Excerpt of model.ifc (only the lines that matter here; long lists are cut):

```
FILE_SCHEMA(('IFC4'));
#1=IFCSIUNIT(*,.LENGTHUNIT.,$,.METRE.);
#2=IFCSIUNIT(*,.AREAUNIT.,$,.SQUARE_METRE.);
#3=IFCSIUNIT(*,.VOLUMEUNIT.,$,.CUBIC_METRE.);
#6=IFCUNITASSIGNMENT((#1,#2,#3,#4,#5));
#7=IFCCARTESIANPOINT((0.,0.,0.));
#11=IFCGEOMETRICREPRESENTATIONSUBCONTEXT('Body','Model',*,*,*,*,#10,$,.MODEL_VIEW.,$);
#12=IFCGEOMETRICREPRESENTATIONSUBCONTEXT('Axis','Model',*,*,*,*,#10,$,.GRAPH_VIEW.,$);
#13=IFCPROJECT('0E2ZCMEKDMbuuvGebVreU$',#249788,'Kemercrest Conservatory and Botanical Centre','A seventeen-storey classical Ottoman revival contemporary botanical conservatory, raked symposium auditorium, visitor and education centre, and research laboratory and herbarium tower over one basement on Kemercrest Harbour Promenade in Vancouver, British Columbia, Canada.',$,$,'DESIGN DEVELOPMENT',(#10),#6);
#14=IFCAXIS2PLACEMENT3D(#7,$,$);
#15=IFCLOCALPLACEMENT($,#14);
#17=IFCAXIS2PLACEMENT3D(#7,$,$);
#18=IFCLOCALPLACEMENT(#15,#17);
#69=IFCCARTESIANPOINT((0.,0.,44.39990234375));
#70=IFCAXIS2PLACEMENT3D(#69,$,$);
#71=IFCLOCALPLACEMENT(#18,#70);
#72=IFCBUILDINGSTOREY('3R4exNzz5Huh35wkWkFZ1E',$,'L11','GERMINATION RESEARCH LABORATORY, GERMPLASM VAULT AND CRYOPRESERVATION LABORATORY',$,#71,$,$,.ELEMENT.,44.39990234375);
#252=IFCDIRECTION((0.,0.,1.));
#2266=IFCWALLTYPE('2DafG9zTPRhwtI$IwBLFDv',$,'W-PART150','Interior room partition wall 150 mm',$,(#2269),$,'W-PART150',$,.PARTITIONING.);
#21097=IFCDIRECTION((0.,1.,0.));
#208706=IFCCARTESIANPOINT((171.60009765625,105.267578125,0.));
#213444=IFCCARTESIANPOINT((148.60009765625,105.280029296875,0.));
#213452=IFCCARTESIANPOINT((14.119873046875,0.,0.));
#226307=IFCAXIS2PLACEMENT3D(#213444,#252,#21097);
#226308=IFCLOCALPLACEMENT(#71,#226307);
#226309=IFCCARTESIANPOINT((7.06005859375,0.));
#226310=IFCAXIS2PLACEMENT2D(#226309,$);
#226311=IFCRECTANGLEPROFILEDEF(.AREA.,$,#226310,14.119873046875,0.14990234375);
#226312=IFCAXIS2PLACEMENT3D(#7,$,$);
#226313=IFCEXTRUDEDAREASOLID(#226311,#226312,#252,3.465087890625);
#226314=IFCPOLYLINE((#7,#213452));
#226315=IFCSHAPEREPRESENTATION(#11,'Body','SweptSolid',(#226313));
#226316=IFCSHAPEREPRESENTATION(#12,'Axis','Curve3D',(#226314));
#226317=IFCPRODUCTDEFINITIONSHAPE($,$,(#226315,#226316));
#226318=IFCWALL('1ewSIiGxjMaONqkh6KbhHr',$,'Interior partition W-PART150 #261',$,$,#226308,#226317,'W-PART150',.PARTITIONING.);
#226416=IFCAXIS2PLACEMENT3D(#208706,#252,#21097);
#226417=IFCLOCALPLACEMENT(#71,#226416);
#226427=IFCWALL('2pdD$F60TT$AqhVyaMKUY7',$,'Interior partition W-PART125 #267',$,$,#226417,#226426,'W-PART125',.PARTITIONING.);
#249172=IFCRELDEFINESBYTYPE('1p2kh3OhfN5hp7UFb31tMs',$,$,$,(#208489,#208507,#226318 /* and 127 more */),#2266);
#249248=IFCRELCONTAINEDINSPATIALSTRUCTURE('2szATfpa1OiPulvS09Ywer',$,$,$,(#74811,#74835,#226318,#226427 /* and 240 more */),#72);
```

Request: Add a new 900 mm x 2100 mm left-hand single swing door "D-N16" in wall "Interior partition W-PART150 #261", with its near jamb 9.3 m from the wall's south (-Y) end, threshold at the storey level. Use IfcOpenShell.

```python
import numpy as np
import ifcopenshell
import ifcopenshell.api.feature
import ifcopenshell.api.geometry
import ifcopenshell.api.root
import ifcopenshell.api.spatial
import ifcopenshell.geom
import ifcopenshell.util.element
import ifcopenshell.util.placement
import ifcopenshell.util.representation
import ifcopenshell.util.shape
import ifcopenshell.util.unit

model = ifcopenshell.open("model.ifc")
unit_scale = ifcopenshell.util.unit.calculate_unit_scale(model)
settings = ifcopenshell.geom.settings()


def volume(element):
    """Net volume in cubic metres, openings subtracted."""
    shape = ifcopenshell.geom.create_shape(settings, element)
    return ifcopenshell.util.shape.get_volume(shape.geometry)


wall = model.by_guid("1ewSIiGxjMaONqkh6KbhHr")
storey = ifcopenshell.util.element.get_container(wall, ifc_class="IfcBuildingStorey")
context = ifcopenshell.util.representation.get_context(model, "Model", "Body", "MODEL_VIEW")
before = volume(wall)

width, height, from_end, sill = 0.9, 2.1, 9.3, 0.0  # metres

# The wall runs along its own X axis, and the end named is its -X end.
wall_shape = ifcopenshell.geom.create_shape(settings, wall)
x, y, z = ifcopenshell.util.shape.get_vertices(wall_shape.geometry).T
start = x.min() + from_end
face, thickness = float(y.min()), float(y.max() - y.min())
wall_matrix = ifcopenshell.util.placement.get_local_placement(wall.ObjectPlacement)
level = ifcopenshell.util.placement.get_local_placement(storey.ObjectPlacement)[2, 3]


def in_wall(x, y):
    """Placement at x, y metres in the wall's axes, at sill height."""
    matrix = wall_matrix.copy()
    matrix[:, 3] = wall_matrix @ np.array([x / unit_scale, y / unit_scale, 0.0, 1.0])
    matrix[2, 3] = level + sill / unit_scale
    return matrix


# Opening: a box that overshoots both wall faces by 50 mm.
opening = ifcopenshell.api.root.create_entity(model, ifc_class="IfcOpeningElement", predefined_type="OPENING")
box = ifcopenshell.api.geometry.add_wall_representation(
    model, context=context, length=width, height=height, thickness=thickness + 0.1
)
ifcopenshell.api.geometry.assign_representation(model, product=opening, representation=box)
ifcopenshell.api.geometry.edit_object_placement(model, product=opening, matrix=in_wall(start, face - 0.05), is_si=False)
ifcopenshell.api.feature.add_feature(model, feature=opening, element=wall)

door = ifcopenshell.api.root.create_entity(model, ifc_class="IfcDoor", name="D-N16", predefined_type="DOOR")
door.OverallWidth, door.OverallHeight = width / unit_scale, height / unit_scale
door.OperationType = "SINGLE_SWING_LEFT"
body = ifcopenshell.api.geometry.add_door_representation(
    model,
    context=context,
    overall_width=door.OverallWidth,
    overall_height=door.OverallHeight,
    operation_type="SINGLE_SWING_LEFT",
    lining_properties={"LiningDepth": thickness / unit_scale, "ThresholdDepth": thickness / unit_scale},
)
ifcopenshell.api.geometry.assign_representation(model, product=door, representation=body)
ifcopenshell.api.spatial.assign_container(model, products=[door], relating_structure=storey)
ifcopenshell.api.feature.add_filling(model, opening=opening, element=door)

# The lining spans the wall, so the door starts at the wall face.
ifcopenshell.api.geometry.edit_object_placement(model, product=door, matrix=in_wall(start, face), is_si=False)

after = volume(wall)

print(f"wall volume {before:.3f} -> {after:.3f} m3")

model.write("model_edited.ifc")
```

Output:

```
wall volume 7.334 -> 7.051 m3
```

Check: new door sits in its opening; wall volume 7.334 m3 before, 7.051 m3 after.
